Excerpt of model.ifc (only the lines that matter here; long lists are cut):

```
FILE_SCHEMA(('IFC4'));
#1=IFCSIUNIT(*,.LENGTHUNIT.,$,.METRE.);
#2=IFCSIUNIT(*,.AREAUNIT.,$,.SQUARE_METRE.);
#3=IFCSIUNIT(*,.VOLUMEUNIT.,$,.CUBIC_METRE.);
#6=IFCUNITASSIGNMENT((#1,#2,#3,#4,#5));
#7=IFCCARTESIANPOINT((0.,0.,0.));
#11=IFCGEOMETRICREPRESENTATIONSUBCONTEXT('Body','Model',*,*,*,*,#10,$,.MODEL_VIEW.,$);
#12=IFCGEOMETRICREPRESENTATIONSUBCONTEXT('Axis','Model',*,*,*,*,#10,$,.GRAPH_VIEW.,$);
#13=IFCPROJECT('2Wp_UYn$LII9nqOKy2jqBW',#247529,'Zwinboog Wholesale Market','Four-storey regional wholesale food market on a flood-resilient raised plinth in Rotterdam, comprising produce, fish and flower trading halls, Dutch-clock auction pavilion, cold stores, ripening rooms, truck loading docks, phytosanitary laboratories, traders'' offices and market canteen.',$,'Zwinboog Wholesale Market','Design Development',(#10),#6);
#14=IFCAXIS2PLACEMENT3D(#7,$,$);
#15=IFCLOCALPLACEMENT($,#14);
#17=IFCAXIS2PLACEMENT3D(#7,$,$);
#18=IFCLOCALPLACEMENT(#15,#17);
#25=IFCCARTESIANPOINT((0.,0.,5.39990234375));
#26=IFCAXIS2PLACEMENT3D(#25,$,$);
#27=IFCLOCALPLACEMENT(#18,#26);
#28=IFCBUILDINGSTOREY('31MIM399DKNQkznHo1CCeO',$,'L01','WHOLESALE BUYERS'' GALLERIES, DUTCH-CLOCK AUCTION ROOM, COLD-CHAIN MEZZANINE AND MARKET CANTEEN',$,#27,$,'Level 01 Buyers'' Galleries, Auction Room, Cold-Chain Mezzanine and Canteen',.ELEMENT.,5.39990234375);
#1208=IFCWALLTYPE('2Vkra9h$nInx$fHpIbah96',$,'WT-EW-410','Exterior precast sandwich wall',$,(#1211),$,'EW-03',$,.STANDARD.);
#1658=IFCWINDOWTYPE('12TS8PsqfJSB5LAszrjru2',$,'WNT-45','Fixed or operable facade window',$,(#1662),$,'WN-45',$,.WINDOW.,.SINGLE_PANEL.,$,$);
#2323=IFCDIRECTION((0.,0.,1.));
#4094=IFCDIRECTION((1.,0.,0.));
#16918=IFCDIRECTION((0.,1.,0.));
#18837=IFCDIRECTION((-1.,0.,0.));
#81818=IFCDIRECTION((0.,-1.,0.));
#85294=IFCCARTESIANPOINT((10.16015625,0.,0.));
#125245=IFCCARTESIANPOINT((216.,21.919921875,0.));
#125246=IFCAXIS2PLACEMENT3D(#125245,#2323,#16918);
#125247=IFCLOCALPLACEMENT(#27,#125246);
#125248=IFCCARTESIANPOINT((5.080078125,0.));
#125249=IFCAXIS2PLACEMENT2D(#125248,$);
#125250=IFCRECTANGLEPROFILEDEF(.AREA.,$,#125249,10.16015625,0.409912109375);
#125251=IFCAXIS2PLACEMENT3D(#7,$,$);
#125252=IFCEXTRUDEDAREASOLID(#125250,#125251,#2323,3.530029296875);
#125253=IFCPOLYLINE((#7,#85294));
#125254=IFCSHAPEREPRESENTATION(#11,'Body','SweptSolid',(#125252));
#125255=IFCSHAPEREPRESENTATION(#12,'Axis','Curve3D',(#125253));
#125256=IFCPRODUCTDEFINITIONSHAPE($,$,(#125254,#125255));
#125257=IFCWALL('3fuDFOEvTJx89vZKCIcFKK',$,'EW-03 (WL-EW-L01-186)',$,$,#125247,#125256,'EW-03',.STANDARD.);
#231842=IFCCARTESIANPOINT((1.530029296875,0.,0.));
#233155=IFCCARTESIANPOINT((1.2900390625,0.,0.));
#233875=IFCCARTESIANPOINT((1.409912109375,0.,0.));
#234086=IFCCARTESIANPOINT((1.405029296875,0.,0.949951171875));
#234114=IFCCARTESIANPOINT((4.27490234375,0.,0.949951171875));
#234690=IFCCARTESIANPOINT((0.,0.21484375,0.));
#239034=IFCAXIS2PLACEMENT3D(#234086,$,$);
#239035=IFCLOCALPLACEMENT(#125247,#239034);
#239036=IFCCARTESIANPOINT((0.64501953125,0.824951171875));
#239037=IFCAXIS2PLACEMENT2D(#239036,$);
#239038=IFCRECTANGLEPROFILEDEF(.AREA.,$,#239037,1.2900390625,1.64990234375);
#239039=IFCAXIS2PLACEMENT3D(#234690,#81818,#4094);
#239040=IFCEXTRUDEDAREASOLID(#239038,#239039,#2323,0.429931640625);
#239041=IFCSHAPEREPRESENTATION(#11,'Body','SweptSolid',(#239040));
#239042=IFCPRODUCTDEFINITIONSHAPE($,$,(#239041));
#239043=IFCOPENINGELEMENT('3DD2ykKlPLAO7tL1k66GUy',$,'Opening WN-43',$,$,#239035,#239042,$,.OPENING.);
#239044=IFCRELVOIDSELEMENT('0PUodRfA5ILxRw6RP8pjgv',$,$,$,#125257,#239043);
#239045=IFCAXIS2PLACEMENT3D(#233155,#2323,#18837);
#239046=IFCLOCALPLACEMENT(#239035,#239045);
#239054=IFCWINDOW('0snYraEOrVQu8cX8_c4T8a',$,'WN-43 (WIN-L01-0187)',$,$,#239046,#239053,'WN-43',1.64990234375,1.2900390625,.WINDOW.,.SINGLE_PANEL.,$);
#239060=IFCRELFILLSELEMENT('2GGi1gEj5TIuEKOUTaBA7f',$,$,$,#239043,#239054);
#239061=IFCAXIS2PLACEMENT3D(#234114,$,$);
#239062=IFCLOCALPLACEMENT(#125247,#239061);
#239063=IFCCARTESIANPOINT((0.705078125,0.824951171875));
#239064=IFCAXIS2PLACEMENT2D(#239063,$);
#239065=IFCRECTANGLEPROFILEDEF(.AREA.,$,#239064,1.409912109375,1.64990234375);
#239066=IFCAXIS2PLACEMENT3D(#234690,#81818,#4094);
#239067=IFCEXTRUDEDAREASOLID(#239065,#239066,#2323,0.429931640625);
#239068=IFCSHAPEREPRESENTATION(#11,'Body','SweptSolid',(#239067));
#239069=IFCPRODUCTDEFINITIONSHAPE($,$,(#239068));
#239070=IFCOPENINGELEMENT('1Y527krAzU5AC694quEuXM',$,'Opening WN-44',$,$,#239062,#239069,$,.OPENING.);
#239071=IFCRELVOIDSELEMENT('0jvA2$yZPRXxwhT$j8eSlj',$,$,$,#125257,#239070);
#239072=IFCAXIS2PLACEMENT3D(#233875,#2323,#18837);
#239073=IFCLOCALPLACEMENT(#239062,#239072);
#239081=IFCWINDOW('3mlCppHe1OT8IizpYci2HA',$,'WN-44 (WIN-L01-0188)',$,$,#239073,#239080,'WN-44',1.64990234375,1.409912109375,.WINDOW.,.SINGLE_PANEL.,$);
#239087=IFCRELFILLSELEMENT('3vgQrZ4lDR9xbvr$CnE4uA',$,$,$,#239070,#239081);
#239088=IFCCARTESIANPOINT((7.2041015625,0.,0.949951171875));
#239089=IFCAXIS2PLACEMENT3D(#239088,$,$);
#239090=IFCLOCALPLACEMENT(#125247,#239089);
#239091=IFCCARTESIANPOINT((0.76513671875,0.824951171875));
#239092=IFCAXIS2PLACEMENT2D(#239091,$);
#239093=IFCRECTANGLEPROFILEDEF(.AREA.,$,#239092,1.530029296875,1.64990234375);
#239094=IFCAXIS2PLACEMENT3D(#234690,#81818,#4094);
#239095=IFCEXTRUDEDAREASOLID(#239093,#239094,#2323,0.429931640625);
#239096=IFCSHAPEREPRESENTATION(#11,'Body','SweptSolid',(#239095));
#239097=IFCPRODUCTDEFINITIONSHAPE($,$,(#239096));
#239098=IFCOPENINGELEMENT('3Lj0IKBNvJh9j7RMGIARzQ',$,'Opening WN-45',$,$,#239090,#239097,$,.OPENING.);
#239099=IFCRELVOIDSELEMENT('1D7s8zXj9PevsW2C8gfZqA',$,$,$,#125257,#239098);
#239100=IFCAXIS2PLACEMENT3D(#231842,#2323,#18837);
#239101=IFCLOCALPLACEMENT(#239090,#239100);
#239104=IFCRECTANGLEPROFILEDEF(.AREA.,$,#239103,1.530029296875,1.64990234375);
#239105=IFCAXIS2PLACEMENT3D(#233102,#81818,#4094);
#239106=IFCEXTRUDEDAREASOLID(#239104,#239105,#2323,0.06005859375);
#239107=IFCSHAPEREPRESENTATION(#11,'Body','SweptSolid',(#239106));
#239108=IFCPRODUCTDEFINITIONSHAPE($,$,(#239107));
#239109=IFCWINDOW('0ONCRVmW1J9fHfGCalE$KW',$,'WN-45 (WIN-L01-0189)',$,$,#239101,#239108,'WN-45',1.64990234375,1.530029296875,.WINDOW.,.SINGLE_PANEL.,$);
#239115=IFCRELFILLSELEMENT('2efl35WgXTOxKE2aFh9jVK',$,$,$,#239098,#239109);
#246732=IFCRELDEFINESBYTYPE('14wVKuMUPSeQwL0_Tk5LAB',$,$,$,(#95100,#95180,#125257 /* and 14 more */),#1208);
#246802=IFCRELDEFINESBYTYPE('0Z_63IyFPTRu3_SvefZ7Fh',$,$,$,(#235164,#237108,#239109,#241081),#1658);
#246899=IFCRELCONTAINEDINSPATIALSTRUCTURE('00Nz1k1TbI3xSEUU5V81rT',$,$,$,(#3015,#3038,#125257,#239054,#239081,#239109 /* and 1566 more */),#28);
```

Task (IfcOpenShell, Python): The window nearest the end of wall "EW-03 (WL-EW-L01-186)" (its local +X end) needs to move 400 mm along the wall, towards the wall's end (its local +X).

```python
import ifcopenshell
import ifcopenshell.api.geometry
import ifcopenshell.util.placement

model = ifcopenshell.open("model.ifc")

window = model.by_id(239109)
opening = window.FillsVoids[0].RelatingOpeningElement
wall = opening.VoidsElements[0].RelatingBuildingElement

wall_matrix = ifcopenshell.util.placement.get_local_placement(wall.ObjectPlacement)
shift = wall_matrix[:3, 0] * 0.4
before = ifcopenshell.util.placement.get_local_placement(window.ObjectPlacement)[:3, 3].copy()

# The window is placed relative to its opening, so it follows when the opening moves.
matrix = ifcopenshell.util.placement.get_local_placement(opening.ObjectPlacement)
matrix[:3, 3] += shift
ifcopenshell.api.geometry.edit_object_placement(
    model, product=opening, matrix=matrix, is_si=False, should_transform_children=True
)

after = ifcopenshell.util.placement.get_local_placement(window.ObjectPlacement)[:3, 3]
print("window moved by", (after - before).round(3) + 0.0)

model.write("model_v2.ifc")
```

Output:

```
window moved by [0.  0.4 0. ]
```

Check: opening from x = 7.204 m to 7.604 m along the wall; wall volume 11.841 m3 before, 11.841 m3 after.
